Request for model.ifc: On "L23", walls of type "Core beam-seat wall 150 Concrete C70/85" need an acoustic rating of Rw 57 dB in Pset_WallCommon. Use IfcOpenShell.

First a look at what the model holds.

```python
import ifcopenshell
import ifcopenshell.util.element

model = ifcopenshell.open("model.ifc")
print(model.schema)
storey = next(s for s in model.by_type("IfcBuildingStorey") if s.Name == "L23")
walls = [e for e in ifcopenshell.util.element.get_decomposition(storey) if e.is_a("IfcWall")]
seen = {}
for e in walls:
    element_type = ifcopenshell.util.element.get_type(e)
    key = (element_type.Name if element_type != e and element_type else None, ifcopenshell.util.element.get_pset(e, "Pset_WallCommon", "AcousticRating"))
    seen[key] = seen.get(key, 0) + 1
for (name, value), count in sorted(seen.items(), key=str):
    print(count, "x", name, "|", value)
```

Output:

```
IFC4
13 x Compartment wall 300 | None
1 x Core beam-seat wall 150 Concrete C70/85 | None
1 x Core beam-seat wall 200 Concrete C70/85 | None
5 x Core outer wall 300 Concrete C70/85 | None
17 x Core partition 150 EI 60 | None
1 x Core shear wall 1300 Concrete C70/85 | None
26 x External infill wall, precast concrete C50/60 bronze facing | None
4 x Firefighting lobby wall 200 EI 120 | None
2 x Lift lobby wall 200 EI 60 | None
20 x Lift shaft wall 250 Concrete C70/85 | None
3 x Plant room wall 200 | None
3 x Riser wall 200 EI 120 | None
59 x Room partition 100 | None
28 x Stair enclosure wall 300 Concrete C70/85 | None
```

```python
import ifcopenshell
import ifcopenshell.api.pset
import ifcopenshell.util.element

model = ifcopenshell.open("model.ifc")

storey = next(s for s in model.by_type("IfcBuildingStorey") if s.Name == "L23")
walls = [e for e in ifcopenshell.util.element.get_decomposition(storey) if e.is_a("IfcWall")]

count = 0
for e in walls:
    element_type = ifcopenshell.util.element.get_type(e)
    if element_type in (None, e) or element_type.Name != "Core beam-seat wall 150 Concrete C70/85":
        continue
    found = ifcopenshell.util.element.get_pset(e, "Pset_WallCommon", should_inherit=False)
    if found:
        pset = model.by_id(found["id"])
        if len(ifcopenshell.util.element.get_elements_by_pset(pset)) > 1:
            pset = ifcopenshell.api.pset.unshare_pset(model, products=[e], pset=pset)[0]
    else:
        pset = ifcopenshell.api.pset.add_pset(model, product=e, name="Pset_WallCommon")
    ifcopenshell.api.pset.edit_pset(model, pset=pset, properties={"AcousticRating": "Rw 57 dB"})
    count += 1

print(count, "walls updated")

model.write("model_rev.ifc")
```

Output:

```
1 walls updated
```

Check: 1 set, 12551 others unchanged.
